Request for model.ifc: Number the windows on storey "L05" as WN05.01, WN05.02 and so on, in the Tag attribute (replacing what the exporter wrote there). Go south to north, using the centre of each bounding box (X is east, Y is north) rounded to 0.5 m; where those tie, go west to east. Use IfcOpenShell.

First a look at what the model holds.

```python
import ifcopenshell
import ifcopenshell.util.element
import ifcopenshell.util.placement

model = ifcopenshell.open("model.ifc")
print(model.schema)
storey = next(s for s in model.by_type("IfcBuildingStorey") if s.Name == "L05")
windows = [e for e in ifcopenshell.util.element.get_decomposition(storey) if e.is_a("IfcWindow")]
for e in sorted(windows, key=lambda e: e.id()):
    origin = ifcopenshell.util.placement.get_local_placement(e.ObjectPlacement)[:3, 3]
    print(e.id(), e.Tag, e.Name, origin.round(2) + 0.0, sep=" | ")
```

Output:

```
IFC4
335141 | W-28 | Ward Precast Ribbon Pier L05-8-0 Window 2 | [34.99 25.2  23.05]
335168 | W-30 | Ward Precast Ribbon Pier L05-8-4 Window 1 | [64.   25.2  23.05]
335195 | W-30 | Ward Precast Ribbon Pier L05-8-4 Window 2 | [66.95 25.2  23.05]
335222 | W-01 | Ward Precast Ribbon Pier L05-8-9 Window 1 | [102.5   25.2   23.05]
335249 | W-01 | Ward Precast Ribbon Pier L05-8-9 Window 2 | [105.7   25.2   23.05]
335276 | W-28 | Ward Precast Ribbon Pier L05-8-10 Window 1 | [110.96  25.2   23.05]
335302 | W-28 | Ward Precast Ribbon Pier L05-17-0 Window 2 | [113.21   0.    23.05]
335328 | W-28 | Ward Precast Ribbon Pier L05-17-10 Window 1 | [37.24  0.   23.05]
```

```python
import ifcopenshell
import ifcopenshell.geom
import ifcopenshell.util.element
import ifcopenshell.util.shape

model = ifcopenshell.open("model.ifc")
settings = ifcopenshell.geom.settings()
settings.set("use-world-coords", True)


def centre(element):
    shape = ifcopenshell.geom.create_shape(settings, element)
    return ifcopenshell.util.shape.get_bbox_centroid(shape.geometry)


storey = next(s for s in model.by_type("IfcBuildingStorey") if s.Name == "L05")
windows = [e for e in ifcopenshell.util.element.get_decomposition(storey) if e.is_a("IfcWindow")]

# Insertion points can sit at a corner or the storey origin, so sort by the geometry (in metres).
centres = {e: centre(e) for e in windows}
windows.sort(key=lambda e: (round(centres[e][1] / 0.5), centres[e][0]))

for i, e in enumerate(windows, start=1):
    number = f"WN05.{i:02d}"
    e.Tag = number
    print(e.id(), number)

model.write("model_rev.ifc")
```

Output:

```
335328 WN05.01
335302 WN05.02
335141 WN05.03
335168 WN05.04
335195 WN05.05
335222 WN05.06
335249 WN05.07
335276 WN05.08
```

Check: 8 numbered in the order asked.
